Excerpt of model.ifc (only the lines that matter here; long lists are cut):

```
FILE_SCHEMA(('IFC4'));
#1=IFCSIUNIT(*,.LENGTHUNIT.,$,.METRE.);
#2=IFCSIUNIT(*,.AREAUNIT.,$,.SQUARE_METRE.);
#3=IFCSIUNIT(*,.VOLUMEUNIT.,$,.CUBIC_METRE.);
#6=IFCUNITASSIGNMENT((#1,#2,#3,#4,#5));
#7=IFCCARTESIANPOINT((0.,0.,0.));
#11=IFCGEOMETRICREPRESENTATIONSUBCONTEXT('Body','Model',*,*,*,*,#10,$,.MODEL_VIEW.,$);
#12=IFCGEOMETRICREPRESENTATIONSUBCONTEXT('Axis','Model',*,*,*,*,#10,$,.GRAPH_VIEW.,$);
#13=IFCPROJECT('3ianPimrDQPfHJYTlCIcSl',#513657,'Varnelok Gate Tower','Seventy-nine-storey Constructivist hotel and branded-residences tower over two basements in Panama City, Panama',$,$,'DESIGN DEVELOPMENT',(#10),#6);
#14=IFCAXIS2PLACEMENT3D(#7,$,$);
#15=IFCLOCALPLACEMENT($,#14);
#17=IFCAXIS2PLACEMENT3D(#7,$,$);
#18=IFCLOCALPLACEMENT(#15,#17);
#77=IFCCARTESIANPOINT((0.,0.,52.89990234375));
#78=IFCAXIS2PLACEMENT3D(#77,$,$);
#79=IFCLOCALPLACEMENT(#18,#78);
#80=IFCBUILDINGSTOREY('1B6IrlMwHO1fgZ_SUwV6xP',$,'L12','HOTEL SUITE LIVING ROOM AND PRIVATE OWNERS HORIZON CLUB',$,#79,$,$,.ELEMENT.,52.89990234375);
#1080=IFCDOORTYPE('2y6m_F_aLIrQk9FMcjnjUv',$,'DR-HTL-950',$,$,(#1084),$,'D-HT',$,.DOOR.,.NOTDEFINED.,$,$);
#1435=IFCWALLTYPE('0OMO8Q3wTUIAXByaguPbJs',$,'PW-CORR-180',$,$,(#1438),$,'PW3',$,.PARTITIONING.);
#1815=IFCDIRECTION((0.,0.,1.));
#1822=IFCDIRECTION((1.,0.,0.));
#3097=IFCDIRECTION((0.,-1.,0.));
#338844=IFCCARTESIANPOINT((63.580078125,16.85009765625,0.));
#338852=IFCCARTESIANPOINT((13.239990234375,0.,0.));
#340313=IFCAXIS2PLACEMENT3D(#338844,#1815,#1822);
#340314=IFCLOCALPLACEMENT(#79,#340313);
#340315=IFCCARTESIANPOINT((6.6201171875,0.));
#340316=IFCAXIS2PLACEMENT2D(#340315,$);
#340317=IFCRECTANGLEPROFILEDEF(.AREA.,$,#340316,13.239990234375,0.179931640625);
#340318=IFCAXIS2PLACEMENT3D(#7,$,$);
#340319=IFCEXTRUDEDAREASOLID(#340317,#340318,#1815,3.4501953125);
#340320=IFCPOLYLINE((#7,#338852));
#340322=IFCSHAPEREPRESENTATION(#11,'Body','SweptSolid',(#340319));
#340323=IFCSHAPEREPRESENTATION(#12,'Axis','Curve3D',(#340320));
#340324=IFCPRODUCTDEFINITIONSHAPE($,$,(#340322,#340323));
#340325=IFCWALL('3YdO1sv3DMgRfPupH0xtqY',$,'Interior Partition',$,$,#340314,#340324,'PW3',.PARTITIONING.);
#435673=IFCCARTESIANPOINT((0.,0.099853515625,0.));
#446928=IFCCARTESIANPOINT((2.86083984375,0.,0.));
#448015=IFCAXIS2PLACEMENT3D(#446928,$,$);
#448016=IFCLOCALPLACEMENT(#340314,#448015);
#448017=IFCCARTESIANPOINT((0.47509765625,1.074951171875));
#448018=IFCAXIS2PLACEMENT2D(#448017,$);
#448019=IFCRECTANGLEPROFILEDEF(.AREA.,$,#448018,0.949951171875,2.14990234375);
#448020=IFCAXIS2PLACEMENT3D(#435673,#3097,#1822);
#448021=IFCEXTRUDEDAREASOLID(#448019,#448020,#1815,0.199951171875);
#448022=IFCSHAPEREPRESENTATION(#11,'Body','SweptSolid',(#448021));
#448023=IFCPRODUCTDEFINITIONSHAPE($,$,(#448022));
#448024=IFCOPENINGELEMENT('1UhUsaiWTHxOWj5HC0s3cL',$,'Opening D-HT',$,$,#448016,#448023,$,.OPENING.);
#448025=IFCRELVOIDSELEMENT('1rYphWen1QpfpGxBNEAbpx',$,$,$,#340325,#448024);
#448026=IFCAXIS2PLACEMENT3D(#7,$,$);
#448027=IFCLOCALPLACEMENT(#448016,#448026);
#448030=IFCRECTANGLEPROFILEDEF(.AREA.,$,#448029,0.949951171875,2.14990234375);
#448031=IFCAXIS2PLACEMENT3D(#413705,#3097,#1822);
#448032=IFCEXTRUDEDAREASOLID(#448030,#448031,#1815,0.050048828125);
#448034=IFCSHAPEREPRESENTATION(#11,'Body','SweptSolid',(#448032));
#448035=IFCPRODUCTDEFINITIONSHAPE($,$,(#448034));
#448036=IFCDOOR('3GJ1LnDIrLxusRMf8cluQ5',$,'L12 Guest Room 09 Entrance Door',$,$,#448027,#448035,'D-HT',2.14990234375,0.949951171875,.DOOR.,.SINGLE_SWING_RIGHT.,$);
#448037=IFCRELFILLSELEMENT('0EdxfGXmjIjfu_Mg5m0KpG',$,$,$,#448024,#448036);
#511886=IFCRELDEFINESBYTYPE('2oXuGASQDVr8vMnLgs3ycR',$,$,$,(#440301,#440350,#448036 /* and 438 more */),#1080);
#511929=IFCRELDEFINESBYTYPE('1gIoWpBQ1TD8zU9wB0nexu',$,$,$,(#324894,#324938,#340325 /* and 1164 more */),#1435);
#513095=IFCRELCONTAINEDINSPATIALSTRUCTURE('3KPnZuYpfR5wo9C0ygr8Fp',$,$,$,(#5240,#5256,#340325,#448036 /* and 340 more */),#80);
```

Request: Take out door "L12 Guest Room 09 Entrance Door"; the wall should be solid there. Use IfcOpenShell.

```python
import ifcopenshell
import ifcopenshell.api.feature
import ifcopenshell.api.root
import ifcopenshell.geom
import ifcopenshell.util.shape

model = ifcopenshell.open("model.ifc")
settings = ifcopenshell.geom.settings()


def volume(element):
    """Net volume in cubic metres, openings subtracted."""
    shape = ifcopenshell.geom.create_shape(settings, element)
    return ifcopenshell.util.shape.get_volume(shape.geometry)


door = model.by_id(448036)
opening = door.FillsVoids[0].RelatingOpeningElement
wall = opening.VoidsElements[0].RelatingBuildingElement
before = volume(wall)

ifcopenshell.api.root.remove_product(model, product=door)
ifcopenshell.api.feature.remove_feature(model, feature=opening)

after = volume(wall)

print(f"wall volume {before:.3f} -> {after:.3f} m3")

model.write("model_v2.ifc")
```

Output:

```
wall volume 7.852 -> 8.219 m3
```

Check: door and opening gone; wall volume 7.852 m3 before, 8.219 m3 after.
